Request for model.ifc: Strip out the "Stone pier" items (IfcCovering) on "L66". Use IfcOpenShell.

First a look at what the model holds.

```python
import ifcopenshell
import ifcopenshell.util.element

model = ifcopenshell.open("model.ifc")
print(model.schema)
storey = next(s for s in model.by_type("IfcBuildingStorey") if s.Name == "L66")
coverings = [e for e in ifcopenshell.util.element.get_decomposition(storey) if e.is_a("IfcCovering")]
seen = {}
for e in coverings:
    element_type = ifcopenshell.util.element.get_type(e)
    name = element_type.Name if element_type not in (None, e) else None
    seen[name] = seen.get(name, 0) + 1
for name, count in sorted(seen.items(), key=str):
    print(count, "x", name)
```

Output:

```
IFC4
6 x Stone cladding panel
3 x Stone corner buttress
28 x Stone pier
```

```python
import ifcopenshell
import ifcopenshell.api.root
import ifcopenshell.util.element

model = ifcopenshell.open("model.ifc")

storey = next(s for s in model.by_type("IfcBuildingStorey") if s.Name == "L66")
coverings = [e for e in ifcopenshell.util.element.get_decomposition(storey) if e.is_a("IfcCovering")]
targets = [e for e in coverings if (t := ifcopenshell.util.element.get_type(e)) not in (None, e) and t.Name == "Stone pier"]

for e in targets:
    ifcopenshell.api.root.remove_product(model, product=e)
print(len(targets), "removed")

model.write("model_updated.ifc")
```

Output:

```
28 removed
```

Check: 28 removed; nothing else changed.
